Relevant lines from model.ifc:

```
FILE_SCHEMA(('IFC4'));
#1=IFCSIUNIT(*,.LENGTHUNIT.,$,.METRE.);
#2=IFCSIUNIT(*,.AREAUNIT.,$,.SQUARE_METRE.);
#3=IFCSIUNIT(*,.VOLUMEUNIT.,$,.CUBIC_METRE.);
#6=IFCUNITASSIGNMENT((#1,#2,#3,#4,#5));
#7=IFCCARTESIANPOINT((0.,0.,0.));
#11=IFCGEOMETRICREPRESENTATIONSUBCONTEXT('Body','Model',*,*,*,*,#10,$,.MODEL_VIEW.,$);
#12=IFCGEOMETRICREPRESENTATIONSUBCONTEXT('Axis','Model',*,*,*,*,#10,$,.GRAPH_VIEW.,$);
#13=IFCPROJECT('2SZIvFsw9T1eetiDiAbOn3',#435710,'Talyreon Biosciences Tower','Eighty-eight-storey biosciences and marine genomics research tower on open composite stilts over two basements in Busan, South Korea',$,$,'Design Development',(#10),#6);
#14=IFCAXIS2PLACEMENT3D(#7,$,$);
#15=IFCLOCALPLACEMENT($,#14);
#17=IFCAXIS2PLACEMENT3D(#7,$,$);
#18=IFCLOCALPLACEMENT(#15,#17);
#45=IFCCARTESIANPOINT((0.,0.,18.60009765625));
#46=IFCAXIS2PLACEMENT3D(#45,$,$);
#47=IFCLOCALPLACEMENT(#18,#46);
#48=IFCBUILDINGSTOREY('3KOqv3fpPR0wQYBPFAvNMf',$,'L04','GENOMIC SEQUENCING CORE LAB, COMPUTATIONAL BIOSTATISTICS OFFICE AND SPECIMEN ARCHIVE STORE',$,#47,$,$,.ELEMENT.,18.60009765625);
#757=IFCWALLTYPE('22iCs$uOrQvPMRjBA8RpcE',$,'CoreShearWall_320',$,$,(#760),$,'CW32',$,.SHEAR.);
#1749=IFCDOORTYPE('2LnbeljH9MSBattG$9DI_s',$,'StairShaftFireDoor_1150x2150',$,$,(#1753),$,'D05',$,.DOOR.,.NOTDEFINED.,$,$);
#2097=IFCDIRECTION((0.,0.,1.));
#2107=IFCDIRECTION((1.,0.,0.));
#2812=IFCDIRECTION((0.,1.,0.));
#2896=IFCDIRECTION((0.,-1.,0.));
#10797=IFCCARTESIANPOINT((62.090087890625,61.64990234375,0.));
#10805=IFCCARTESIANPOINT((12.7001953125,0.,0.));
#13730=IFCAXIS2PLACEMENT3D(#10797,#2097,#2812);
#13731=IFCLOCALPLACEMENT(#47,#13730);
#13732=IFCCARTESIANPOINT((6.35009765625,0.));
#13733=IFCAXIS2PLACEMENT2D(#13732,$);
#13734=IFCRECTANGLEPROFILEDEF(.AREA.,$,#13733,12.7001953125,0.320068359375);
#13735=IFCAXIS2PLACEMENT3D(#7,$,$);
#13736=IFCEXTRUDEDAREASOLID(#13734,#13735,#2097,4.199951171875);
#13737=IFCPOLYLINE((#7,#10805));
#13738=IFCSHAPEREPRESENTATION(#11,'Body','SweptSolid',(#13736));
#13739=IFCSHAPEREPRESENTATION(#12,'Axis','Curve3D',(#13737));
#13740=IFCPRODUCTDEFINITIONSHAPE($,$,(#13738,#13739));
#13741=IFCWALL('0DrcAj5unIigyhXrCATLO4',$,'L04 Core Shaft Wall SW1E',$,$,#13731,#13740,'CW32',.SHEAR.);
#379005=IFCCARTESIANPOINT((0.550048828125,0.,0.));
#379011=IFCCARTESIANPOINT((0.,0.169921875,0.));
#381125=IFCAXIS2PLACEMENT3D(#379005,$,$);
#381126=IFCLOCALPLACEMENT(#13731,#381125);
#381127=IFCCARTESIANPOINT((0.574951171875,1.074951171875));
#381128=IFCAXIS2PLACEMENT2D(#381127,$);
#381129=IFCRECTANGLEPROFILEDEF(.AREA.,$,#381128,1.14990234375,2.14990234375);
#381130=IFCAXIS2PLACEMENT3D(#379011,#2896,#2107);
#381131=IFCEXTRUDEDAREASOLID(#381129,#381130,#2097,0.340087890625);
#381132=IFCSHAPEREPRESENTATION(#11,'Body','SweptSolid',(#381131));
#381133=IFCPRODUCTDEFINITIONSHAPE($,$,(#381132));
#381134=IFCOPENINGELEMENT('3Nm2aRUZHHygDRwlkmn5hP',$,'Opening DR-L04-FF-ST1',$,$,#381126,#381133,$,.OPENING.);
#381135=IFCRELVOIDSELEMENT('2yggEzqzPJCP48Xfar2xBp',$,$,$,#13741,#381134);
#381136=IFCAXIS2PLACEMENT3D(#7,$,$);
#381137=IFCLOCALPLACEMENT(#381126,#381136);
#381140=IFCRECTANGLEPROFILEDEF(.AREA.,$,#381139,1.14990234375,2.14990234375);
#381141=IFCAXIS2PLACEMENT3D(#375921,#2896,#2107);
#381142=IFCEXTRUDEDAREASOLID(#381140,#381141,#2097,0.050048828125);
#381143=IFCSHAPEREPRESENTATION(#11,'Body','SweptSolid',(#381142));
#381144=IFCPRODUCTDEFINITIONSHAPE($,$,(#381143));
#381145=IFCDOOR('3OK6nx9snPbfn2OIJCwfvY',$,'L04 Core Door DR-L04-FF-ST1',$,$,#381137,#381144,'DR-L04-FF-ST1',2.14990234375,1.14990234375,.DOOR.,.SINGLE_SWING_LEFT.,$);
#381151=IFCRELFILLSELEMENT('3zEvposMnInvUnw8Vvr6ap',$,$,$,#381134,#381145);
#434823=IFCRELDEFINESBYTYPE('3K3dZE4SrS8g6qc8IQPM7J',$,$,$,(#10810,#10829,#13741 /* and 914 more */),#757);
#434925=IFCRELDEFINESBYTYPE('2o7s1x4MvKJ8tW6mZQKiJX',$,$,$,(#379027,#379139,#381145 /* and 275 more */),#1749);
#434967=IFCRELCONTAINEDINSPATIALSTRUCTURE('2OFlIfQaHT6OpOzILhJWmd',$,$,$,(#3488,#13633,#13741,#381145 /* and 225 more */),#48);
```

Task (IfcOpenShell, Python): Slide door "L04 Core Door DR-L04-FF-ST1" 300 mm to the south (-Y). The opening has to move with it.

```python
import ifcopenshell
import ifcopenshell.api.geometry
import ifcopenshell.util.placement
import ifcopenshell.util.unit

model = ifcopenshell.open("model.ifc")
unit_scale = ifcopenshell.util.unit.calculate_unit_scale(model)

door = model.by_guid("3OK6nx9snPbfn2OIJCwfvY")
opening = door.FillsVoids[0].RelatingOpeningElement
wall = opening.VoidsElements[0].RelatingBuildingElement

wall_matrix = ifcopenshell.util.placement.get_local_placement(wall.ObjectPlacement)
shift = wall_matrix[:3, 0] * -0.3 / unit_scale
before = ifcopenshell.util.placement.get_local_placement(door.ObjectPlacement)[:3, 3].copy()

# The door is placed relative to its opening, so it follows when the opening moves.
matrix = ifcopenshell.util.placement.get_local_placement(opening.ObjectPlacement)
matrix[:3, 3] += shift
ifcopenshell.api.geometry.edit_object_placement(
    model, product=opening, matrix=matrix, is_si=False, should_transform_children=True
)

after = ifcopenshell.util.placement.get_local_placement(door.ObjectPlacement)[:3, 3]
print("door moved by", (after - before).round(3) + 0.0)

model.write("model-out.ifc")
```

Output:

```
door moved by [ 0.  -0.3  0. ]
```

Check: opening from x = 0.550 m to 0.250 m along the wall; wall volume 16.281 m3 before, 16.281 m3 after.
